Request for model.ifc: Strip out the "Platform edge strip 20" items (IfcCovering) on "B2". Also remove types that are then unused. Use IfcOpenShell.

First a look at what the model holds.

```python
import ifcopenshell
import ifcopenshell.util.element

model = ifcopenshell.open("model.ifc")
print(model.schema)
storey = next(s for s in model.by_type("IfcBuildingStorey") if s.Name == "B2")
coverings = [e for e in ifcopenshell.util.element.get_decomposition(storey) if e.is_a("IfcCovering")]
seen = {}
for e in coverings:
    element_type = ifcopenshell.util.element.get_type(e)
    name = element_type.Name if element_type not in (None, e) else None
    seen[name] = seen.get(name, 0) + 1
for name, count in sorted(seen.items(), key=str):
    print(count, "x", name)
```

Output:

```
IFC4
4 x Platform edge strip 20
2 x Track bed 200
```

```python
import ifcopenshell
import ifcopenshell.api.root
import ifcopenshell.util.element

model = ifcopenshell.open("model.ifc")

storey = next(s for s in model.by_type("IfcBuildingStorey") if s.Name == "B2")
coverings = [e for e in ifcopenshell.util.element.get_decomposition(storey) if e.is_a("IfcCovering")]
targets = [e for e in coverings if (t := ifcopenshell.util.element.get_type(e)) not in (None, e) and t.Name == "Platform edge strip 20"]
types = {ifcopenshell.util.element.get_type(e) for e in targets} - {None, *targets}

for e in targets:
    ifcopenshell.api.root.remove_product(model, product=e)
print(len(targets), "removed")

unused = [t for t in types if not ifcopenshell.util.element.get_types(t)]
for t in unused:
    ifcopenshell.api.root.remove_product(model, product=t)
print(len(unused), "unused types removed")

model.write("model-out.ifc")
```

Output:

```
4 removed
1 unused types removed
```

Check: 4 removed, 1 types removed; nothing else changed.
